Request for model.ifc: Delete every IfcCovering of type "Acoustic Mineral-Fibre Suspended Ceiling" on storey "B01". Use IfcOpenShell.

First a look at what the model holds.

```python
import ifcopenshell
import ifcopenshell.util.element

model = ifcopenshell.open("model.ifc")
print(model.schema)
storey = next(s for s in model.by_type("IfcBuildingStorey") if s.Name == "B01")
coverings = [e for e in ifcopenshell.util.element.get_decomposition(storey) if e.is_a("IfcCovering")]
seen = {}
for e in coverings:
    element_type = ifcopenshell.util.element.get_type(e)
    name = element_type.Name if element_type not in (None, e) else None
    seen[name] = seen.get(name, 0) + 1
for name, count in sorted(seen.items(), key=str):
    print(count, "x", name)
```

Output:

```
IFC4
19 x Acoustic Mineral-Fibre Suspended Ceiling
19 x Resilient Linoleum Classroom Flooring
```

```python
import ifcopenshell
import ifcopenshell.api.root
import ifcopenshell.util.element

model = ifcopenshell.open("model.ifc")

storey = next(s for s in model.by_type("IfcBuildingStorey") if s.Name == "B01")
coverings = [e for e in ifcopenshell.util.element.get_decomposition(storey) if e.is_a("IfcCovering")]
targets = [e for e in coverings if (t := ifcopenshell.util.element.get_type(e)) not in (None, e) and t.Name == "Acoustic Mineral-Fibre Suspended Ceiling"]

for e in targets:
    ifcopenshell.api.root.remove_product(model, product=e)
print(len(targets), "removed")

model.write("model_rev.ifc")
```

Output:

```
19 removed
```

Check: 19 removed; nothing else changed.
